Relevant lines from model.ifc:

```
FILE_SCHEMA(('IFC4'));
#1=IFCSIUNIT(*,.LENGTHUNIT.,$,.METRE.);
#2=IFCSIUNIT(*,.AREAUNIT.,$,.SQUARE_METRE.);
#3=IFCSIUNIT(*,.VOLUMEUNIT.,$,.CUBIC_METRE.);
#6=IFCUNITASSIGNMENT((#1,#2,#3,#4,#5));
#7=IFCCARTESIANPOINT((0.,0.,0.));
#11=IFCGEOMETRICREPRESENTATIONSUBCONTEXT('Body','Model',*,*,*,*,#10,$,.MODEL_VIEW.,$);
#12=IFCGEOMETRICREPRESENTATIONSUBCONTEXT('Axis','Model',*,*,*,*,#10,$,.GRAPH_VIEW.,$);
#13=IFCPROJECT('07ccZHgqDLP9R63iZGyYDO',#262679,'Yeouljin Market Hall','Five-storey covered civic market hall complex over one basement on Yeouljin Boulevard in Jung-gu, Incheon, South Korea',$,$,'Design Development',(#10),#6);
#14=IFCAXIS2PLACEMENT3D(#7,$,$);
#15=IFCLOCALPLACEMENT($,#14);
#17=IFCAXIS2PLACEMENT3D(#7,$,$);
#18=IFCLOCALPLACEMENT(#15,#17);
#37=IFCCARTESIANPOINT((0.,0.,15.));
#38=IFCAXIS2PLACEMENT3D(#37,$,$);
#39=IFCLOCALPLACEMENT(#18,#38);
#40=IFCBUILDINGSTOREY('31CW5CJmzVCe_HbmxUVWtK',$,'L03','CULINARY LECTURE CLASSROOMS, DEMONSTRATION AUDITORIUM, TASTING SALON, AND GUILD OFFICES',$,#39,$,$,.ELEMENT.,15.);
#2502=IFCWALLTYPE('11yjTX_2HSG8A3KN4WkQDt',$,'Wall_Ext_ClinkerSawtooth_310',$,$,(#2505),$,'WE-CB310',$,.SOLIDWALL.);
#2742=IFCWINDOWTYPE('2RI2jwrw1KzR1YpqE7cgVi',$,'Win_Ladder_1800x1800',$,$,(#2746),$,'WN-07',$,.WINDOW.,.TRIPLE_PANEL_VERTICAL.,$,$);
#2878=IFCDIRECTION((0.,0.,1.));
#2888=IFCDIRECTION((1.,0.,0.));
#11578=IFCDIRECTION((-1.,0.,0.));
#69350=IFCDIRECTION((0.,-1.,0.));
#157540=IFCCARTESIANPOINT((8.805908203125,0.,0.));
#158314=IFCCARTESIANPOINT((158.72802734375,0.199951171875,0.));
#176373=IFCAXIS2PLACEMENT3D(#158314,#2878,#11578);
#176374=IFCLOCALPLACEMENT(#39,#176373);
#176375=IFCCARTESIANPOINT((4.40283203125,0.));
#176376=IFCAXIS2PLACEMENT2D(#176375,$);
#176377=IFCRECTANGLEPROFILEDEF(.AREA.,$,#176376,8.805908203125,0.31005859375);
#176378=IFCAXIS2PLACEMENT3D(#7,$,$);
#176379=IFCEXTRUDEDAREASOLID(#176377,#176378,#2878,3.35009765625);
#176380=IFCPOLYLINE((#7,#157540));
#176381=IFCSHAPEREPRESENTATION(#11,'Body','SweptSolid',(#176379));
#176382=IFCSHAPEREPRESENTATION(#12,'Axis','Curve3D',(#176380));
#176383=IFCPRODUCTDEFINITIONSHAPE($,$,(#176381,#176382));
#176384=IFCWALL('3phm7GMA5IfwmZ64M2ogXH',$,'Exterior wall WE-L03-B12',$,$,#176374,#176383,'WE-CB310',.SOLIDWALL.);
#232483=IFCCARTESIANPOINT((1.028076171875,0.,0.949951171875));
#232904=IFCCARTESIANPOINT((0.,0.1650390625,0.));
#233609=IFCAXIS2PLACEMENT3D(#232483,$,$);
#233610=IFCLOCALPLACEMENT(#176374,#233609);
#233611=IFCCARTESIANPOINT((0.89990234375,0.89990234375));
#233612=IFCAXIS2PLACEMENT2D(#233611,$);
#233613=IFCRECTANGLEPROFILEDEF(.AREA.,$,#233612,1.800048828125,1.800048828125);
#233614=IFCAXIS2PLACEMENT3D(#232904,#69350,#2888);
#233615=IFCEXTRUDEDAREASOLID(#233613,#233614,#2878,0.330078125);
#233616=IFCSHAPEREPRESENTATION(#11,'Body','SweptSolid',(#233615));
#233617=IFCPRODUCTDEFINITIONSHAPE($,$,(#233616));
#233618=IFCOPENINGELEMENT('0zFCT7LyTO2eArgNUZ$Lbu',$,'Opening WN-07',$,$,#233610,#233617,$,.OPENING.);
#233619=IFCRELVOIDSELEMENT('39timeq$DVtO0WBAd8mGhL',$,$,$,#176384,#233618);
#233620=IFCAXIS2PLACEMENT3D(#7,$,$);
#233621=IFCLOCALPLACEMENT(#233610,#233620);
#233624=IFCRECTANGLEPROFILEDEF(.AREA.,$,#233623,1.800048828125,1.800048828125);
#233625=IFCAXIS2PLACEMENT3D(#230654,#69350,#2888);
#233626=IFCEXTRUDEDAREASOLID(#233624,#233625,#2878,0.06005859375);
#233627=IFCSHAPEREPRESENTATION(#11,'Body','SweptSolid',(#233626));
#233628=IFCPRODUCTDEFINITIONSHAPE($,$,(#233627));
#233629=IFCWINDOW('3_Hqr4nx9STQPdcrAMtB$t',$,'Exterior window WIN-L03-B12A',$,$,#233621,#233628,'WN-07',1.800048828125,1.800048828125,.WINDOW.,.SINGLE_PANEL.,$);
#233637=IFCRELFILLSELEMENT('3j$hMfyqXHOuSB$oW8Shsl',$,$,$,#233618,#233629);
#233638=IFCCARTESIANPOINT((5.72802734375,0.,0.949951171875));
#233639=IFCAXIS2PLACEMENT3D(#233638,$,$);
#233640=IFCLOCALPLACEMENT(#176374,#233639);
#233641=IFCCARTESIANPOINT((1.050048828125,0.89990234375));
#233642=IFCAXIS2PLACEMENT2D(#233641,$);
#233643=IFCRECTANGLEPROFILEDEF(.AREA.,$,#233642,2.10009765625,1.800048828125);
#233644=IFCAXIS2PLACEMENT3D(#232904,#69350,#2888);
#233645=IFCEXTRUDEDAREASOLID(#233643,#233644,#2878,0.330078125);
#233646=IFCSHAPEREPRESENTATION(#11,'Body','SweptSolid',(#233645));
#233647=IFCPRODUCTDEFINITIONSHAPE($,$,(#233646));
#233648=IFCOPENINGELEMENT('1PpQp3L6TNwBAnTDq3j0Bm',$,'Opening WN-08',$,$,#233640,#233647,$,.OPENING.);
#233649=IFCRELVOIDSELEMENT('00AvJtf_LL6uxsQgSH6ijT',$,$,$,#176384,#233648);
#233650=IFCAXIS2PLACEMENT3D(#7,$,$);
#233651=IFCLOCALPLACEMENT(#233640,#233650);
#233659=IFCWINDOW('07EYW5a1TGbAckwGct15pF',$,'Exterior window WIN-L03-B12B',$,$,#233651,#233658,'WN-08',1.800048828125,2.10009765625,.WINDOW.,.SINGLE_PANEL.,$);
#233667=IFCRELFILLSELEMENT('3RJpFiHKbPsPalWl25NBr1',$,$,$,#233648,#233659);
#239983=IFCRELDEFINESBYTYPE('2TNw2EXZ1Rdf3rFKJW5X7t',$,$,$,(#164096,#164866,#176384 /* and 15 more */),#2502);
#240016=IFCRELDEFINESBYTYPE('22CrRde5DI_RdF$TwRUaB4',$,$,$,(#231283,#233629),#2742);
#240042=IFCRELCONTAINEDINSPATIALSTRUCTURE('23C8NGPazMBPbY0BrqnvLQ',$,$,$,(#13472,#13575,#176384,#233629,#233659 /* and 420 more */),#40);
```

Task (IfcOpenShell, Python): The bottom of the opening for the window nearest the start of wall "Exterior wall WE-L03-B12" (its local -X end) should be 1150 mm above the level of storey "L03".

```python
import numpy as np
import ifcopenshell
import ifcopenshell.api.geometry
import ifcopenshell.geom
import ifcopenshell.util.element
import ifcopenshell.util.placement
import ifcopenshell.util.shape
import ifcopenshell.util.unit

model = ifcopenshell.open("model.ifc")
unit_scale = ifcopenshell.util.unit.calculate_unit_scale(model)

window = model.by_guid("3_Hqr4nx9STQPdcrAMtB$t")
opening = window.FillsVoids[0].RelatingOpeningElement
storey = ifcopenshell.util.element.get_container(window, ifc_class="IfcBuildingStorey")
level = ifcopenshell.util.placement.get_local_placement(storey.ObjectPlacement)[2, 3]

# The opening's origin need not be at the sill, so measure its lowest point.
shape = ifcopenshell.geom.create_shape(ifcopenshell.geom.settings(), opening)
bottom = ifcopenshell.util.shape.get_shape_bottom_elevation(shape, shape.geometry) / unit_scale
dz = level + 1.15 / unit_scale - bottom

shift = np.array([0.0, 0.0, dz])
# The window is placed relative to its opening, so it follows when the opening moves.
matrix = ifcopenshell.util.placement.get_local_placement(opening.ObjectPlacement)
matrix[:3, 3] += shift
ifcopenshell.api.geometry.edit_object_placement(
    model, product=opening, matrix=matrix, is_si=False, should_transform_children=True
)

print(f"moved by {dz * unit_scale:+.3f} m")

model.write("model_updated.ifc")
```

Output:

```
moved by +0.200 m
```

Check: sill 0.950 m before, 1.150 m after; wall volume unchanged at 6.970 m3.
